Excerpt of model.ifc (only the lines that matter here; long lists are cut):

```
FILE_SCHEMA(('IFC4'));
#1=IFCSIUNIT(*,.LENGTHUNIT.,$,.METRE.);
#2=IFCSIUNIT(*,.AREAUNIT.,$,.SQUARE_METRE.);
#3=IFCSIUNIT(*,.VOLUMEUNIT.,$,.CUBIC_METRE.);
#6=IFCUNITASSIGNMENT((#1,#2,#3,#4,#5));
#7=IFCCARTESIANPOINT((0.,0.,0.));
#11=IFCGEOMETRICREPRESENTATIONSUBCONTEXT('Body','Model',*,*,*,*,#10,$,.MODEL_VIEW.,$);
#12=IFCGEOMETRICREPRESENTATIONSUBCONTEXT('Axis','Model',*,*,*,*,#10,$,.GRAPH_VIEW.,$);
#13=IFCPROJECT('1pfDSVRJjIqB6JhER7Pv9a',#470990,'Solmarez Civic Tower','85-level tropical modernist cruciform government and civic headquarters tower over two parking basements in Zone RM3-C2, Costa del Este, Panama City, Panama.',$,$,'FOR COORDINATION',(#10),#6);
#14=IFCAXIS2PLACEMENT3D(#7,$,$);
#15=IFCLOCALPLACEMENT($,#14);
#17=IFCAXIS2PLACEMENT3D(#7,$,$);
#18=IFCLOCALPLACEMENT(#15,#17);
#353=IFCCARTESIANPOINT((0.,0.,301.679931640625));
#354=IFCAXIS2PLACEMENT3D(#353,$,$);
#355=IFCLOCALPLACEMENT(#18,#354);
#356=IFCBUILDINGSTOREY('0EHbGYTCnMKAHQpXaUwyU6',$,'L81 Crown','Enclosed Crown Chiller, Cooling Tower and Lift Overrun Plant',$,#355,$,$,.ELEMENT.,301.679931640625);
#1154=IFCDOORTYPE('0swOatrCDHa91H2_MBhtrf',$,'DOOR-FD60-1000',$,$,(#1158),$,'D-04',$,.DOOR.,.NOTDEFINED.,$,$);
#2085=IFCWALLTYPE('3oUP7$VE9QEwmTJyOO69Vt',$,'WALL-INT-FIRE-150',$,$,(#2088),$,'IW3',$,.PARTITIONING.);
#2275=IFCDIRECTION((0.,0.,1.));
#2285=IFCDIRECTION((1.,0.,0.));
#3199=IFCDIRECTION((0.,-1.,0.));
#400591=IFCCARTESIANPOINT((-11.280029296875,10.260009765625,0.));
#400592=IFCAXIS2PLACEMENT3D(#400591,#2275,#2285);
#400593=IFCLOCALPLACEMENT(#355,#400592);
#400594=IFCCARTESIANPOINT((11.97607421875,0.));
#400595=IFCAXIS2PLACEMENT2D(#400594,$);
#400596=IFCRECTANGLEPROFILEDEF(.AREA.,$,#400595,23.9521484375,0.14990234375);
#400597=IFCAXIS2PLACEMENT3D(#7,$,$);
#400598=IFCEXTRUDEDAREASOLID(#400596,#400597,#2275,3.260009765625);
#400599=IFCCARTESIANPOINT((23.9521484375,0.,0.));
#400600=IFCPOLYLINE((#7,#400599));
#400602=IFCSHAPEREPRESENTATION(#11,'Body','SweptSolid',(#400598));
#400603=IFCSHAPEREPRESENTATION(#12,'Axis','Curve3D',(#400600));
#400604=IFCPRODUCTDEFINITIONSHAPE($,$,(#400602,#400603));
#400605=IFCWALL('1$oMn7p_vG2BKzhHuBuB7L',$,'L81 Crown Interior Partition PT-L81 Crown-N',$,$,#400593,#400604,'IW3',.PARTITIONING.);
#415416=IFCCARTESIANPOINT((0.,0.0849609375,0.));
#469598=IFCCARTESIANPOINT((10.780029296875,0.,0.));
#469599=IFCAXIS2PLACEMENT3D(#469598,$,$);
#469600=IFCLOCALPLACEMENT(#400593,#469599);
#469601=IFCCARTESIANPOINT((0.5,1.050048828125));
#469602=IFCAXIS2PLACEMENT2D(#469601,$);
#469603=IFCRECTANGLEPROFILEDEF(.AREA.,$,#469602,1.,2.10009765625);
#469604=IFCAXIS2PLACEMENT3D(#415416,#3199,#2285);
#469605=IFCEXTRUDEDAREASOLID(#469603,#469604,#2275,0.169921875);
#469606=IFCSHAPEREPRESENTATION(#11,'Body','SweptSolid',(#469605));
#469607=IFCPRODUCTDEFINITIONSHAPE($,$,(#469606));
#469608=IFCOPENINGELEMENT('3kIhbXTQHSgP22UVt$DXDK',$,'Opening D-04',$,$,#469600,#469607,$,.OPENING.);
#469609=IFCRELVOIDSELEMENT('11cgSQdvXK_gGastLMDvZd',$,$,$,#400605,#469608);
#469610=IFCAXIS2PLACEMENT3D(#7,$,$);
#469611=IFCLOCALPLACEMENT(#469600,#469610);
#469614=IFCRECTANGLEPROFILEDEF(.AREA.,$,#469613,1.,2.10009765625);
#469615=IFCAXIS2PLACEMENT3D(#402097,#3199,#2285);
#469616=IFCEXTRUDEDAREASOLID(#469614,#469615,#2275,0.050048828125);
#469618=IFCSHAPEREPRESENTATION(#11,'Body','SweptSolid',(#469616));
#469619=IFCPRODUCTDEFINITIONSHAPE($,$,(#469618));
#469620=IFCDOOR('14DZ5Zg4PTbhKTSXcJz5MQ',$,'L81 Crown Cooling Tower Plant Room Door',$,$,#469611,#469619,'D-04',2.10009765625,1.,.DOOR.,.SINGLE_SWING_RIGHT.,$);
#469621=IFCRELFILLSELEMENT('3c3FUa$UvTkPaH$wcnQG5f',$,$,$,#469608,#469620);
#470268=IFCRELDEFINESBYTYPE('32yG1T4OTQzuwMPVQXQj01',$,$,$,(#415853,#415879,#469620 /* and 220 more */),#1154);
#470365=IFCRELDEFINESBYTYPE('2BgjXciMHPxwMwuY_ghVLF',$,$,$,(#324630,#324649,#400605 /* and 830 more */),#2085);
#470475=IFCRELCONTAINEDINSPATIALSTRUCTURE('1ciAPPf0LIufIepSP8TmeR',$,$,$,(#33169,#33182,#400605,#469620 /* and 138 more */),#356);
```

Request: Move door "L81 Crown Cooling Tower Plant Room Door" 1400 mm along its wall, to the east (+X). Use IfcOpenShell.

```python
import ifcopenshell
import ifcopenshell.api.geometry
import ifcopenshell.util.placement

model = ifcopenshell.open("model.ifc")

door = model.by_guid("14DZ5Zg4PTbhKTSXcJz5MQ")
opening = door.FillsVoids[0].RelatingOpeningElement
wall = opening.VoidsElements[0].RelatingBuildingElement

wall_matrix = ifcopenshell.util.placement.get_local_placement(wall.ObjectPlacement)
shift = wall_matrix[:3, 0] * 1.4
before = ifcopenshell.util.placement.get_local_placement(door.ObjectPlacement)[:3, 3].copy()

# The door is placed relative to its opening, so it follows when the opening moves.
matrix = ifcopenshell.util.placement.get_local_placement(opening.ObjectPlacement)
matrix[:3, 3] += shift
ifcopenshell.api.geometry.edit_object_placement(
    model, product=opening, matrix=matrix, is_si=False, should_transform_children=True
)

after = ifcopenshell.util.placement.get_local_placement(door.ObjectPlacement)[:3, 3]
print("door moved by", (after - before).round(3) + 0.0)

model.write("model_rev.ifc")
```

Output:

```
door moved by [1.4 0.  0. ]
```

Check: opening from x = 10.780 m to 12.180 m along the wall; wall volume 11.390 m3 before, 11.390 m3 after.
